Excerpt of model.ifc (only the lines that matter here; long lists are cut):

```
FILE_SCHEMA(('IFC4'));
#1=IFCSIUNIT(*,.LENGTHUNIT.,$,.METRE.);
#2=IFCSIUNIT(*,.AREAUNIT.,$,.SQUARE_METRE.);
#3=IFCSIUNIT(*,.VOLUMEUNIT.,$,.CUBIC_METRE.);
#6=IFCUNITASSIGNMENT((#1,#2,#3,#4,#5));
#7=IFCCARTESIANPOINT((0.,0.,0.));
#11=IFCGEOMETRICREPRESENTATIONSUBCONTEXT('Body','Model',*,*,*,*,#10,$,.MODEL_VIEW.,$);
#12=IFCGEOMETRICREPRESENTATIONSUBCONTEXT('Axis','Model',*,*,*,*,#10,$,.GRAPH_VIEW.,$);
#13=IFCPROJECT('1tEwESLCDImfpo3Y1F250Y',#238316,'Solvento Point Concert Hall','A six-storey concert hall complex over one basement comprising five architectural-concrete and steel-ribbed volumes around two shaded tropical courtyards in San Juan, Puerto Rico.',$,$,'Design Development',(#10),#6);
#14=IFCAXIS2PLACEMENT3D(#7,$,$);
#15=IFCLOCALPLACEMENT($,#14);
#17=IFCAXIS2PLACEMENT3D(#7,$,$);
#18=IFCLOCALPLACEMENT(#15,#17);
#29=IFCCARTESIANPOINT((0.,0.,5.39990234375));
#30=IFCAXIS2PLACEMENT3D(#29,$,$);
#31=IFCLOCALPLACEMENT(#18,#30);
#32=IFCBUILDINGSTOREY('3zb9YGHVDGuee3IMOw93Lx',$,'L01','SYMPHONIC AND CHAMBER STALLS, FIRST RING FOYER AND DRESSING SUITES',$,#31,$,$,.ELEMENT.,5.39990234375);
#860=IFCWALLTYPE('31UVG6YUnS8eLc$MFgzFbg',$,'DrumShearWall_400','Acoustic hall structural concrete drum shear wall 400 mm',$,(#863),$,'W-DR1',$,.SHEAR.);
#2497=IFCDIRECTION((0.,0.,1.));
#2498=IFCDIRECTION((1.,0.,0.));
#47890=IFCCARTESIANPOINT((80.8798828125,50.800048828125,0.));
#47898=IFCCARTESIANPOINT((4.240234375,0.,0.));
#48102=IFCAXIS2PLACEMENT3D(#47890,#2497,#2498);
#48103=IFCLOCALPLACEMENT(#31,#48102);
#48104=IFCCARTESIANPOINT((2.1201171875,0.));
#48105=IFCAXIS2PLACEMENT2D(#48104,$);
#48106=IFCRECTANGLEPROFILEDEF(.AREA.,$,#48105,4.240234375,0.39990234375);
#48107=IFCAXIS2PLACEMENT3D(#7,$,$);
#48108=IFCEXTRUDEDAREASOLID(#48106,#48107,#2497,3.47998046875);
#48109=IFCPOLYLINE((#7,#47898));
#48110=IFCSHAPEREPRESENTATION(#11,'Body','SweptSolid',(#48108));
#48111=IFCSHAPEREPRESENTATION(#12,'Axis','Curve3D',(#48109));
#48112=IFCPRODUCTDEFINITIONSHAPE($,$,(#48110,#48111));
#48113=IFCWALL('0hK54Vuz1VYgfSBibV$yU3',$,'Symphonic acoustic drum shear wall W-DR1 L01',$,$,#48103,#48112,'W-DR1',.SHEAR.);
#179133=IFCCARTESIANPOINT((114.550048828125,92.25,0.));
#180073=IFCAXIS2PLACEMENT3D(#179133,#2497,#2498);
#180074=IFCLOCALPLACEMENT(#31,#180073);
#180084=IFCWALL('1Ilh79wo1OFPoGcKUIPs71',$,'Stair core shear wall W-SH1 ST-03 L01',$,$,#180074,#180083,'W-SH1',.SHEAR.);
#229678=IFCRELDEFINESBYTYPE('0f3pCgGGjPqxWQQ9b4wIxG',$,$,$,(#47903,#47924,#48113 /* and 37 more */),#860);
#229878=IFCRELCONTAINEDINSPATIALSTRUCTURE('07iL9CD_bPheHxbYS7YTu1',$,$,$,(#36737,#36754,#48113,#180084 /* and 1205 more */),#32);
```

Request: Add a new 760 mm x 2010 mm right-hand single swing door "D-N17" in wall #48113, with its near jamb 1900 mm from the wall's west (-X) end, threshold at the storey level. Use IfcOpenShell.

```python
import numpy as np
import ifcopenshell
import ifcopenshell.api.feature
import ifcopenshell.api.geometry
import ifcopenshell.api.root
import ifcopenshell.api.spatial
import ifcopenshell.geom
import ifcopenshell.util.element
import ifcopenshell.util.placement
import ifcopenshell.util.representation
import ifcopenshell.util.shape
import ifcopenshell.util.unit

model = ifcopenshell.open("model.ifc")
unit_scale = ifcopenshell.util.unit.calculate_unit_scale(model)
settings = ifcopenshell.geom.settings()


def volume(element):
    """Net volume in cubic metres, openings subtracted."""
    shape = ifcopenshell.geom.create_shape(settings, element)
    return ifcopenshell.util.shape.get_volume(shape.geometry)


wall = model.by_guid("0hK54Vuz1VYgfSBibV$yU3")
storey = ifcopenshell.util.element.get_container(wall, ifc_class="IfcBuildingStorey")
context = ifcopenshell.util.representation.get_context(model, "Model", "Body", "MODEL_VIEW")
before = volume(wall)

width, height, from_end, sill = 0.76, 2.01, 1.9, 0.0  # metres

# The wall runs along its own X axis, and the end named is its -X end.
wall_shape = ifcopenshell.geom.create_shape(settings, wall)
x, y, z = ifcopenshell.util.shape.get_vertices(wall_shape.geometry).T
start = x.min() + from_end
face, thickness = float(y.min()), float(y.max() - y.min())
wall_matrix = ifcopenshell.util.placement.get_local_placement(wall.ObjectPlacement)
level = ifcopenshell.util.placement.get_local_placement(storey.ObjectPlacement)[2, 3]


def in_wall(x, y):
    """Placement at x, y metres in the wall's axes, at sill height."""
    matrix = wall_matrix.copy()
    matrix[:, 3] = wall_matrix @ np.array([x / unit_scale, y / unit_scale, 0.0, 1.0])
    matrix[2, 3] = level + sill / unit_scale
    return matrix


# Opening: a box that overshoots both wall faces by 50 mm.
opening = ifcopenshell.api.root.create_entity(model, ifc_class="IfcOpeningElement", predefined_type="OPENING")
box = ifcopenshell.api.geometry.add_wall_representation(
    model, context=context, length=width, height=height, thickness=thickness + 0.1
)
ifcopenshell.api.geometry.assign_representation(model, product=opening, representation=box)
ifcopenshell.api.geometry.edit_object_placement(model, product=opening, matrix=in_wall(start, face - 0.05), is_si=False)
ifcopenshell.api.feature.add_feature(model, feature=opening, element=wall)

door = ifcopenshell.api.root.create_entity(model, ifc_class="IfcDoor", name="D-N17", predefined_type="DOOR")
door.OverallWidth, door.OverallHeight = width / unit_scale, height / unit_scale
door.OperationType = "SINGLE_SWING_RIGHT"
body = ifcopenshell.api.geometry.add_door_representation(
    model,
    context=context,
    overall_width=door.OverallWidth,
    overall_height=door.OverallHeight,
    operation_type="SINGLE_SWING_RIGHT",
    lining_properties={"LiningDepth": thickness / unit_scale, "ThresholdDepth": thickness / unit_scale},
)
ifcopenshell.api.geometry.assign_representation(model, product=door, representation=body)
ifcopenshell.api.spatial.assign_container(model, products=[door], relating_structure=storey)
ifcopenshell.api.feature.add_filling(model, opening=opening, element=door)

# The lining spans the wall, so the door starts at the wall face.
ifcopenshell.api.geometry.edit_object_placement(model, product=door, matrix=in_wall(start, face), is_si=False)

after = volume(wall)

print(f"wall volume {before:.3f} -> {after:.3f} m3")

model.write("model_rev.ifc")
```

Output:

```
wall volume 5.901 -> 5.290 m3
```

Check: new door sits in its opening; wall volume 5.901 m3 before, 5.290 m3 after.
